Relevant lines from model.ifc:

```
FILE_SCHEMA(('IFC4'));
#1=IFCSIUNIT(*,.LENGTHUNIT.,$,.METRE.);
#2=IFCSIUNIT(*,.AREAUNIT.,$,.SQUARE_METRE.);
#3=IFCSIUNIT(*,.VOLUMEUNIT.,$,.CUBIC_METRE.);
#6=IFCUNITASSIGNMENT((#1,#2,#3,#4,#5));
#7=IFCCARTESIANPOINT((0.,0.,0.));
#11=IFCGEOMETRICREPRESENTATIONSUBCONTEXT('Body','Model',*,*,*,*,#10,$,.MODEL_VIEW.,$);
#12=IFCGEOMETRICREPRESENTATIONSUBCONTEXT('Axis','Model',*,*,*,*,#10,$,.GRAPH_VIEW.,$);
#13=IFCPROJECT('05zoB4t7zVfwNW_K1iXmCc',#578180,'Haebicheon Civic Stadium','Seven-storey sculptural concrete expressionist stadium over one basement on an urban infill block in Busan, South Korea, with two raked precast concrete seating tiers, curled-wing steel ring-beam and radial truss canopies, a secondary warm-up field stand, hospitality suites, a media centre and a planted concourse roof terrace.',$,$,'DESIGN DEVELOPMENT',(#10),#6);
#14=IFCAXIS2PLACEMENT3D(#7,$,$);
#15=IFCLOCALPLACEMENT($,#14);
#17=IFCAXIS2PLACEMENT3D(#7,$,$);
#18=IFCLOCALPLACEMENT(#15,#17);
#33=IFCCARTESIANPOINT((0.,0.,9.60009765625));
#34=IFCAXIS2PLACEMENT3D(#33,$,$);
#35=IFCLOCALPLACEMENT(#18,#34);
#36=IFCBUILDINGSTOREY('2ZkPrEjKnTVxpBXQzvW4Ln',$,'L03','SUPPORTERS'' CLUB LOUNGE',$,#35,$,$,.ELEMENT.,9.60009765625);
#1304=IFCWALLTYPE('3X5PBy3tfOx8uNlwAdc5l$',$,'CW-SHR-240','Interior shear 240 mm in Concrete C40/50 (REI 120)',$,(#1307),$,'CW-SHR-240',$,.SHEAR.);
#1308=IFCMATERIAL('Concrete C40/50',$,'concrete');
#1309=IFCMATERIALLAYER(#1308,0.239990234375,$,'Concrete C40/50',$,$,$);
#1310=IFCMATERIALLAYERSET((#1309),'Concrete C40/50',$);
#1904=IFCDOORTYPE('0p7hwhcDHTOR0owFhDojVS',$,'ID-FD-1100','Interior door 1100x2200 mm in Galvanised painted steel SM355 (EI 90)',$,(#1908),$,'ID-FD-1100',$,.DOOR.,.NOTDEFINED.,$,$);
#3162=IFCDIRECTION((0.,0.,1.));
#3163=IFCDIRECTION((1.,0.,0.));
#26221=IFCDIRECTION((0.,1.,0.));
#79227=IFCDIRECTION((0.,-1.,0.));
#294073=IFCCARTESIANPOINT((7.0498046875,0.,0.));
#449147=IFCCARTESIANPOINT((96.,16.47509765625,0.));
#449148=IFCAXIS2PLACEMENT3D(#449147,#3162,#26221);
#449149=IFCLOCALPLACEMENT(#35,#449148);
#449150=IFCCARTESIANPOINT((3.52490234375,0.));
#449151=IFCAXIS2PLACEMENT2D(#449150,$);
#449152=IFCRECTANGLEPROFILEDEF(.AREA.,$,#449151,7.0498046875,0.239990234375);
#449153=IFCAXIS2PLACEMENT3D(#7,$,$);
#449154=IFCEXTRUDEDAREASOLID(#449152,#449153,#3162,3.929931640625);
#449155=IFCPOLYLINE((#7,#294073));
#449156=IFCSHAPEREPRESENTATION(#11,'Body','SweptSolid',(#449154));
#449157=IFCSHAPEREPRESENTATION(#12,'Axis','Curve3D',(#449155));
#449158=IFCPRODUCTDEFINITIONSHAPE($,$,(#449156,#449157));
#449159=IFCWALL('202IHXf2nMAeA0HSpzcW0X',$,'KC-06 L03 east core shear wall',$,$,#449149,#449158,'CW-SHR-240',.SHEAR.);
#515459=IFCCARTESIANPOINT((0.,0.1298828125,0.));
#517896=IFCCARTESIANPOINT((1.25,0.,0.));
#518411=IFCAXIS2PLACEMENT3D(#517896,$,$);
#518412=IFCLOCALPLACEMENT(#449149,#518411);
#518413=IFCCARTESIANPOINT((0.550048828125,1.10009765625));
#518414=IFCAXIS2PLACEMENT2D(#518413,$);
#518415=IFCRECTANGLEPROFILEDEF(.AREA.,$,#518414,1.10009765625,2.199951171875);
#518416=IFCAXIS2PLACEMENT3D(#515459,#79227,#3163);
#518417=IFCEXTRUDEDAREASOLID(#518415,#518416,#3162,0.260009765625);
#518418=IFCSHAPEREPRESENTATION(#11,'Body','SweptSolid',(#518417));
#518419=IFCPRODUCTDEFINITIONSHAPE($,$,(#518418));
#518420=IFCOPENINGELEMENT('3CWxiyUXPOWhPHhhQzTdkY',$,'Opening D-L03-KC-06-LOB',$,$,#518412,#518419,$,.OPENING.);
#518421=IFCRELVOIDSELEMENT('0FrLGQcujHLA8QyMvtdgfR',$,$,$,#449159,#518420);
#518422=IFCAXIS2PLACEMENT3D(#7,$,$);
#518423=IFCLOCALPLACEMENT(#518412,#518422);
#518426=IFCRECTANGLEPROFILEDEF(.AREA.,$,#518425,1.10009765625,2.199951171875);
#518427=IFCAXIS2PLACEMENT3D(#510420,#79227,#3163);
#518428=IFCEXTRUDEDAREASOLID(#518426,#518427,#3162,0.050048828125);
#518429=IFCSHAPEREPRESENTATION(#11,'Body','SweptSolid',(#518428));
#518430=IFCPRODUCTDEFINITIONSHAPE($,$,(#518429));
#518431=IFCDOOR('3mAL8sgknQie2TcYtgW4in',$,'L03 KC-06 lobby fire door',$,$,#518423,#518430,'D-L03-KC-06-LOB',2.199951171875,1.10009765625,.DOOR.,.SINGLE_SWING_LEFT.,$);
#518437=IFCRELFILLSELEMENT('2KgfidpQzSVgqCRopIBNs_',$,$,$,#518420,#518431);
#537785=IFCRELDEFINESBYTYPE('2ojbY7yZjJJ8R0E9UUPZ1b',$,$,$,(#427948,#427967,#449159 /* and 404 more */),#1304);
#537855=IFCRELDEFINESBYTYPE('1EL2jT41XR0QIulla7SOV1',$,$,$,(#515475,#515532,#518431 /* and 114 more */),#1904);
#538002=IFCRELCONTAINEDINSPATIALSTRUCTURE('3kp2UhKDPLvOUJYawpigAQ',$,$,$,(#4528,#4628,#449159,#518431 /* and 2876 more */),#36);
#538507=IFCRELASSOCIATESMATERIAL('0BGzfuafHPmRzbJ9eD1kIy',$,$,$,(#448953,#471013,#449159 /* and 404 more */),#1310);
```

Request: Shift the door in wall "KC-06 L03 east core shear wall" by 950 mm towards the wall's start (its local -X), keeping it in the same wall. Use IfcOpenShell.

```python
import ifcopenshell
import ifcopenshell.api.geometry
import ifcopenshell.util.placement

model = ifcopenshell.open("model.ifc")

door = model.by_guid("3mAL8sgknQie2TcYtgW4in")
opening = door.FillsVoids[0].RelatingOpeningElement
wall = opening.VoidsElements[0].RelatingBuildingElement

wall_matrix = ifcopenshell.util.placement.get_local_placement(wall.ObjectPlacement)
shift = wall_matrix[:3, 0] * -0.95
before = ifcopenshell.util.placement.get_local_placement(door.ObjectPlacement)[:3, 3].copy()

# The door is placed relative to its opening, so it follows when the opening moves.
matrix = ifcopenshell.util.placement.get_local_placement(opening.ObjectPlacement)
matrix[:3, 3] += shift
ifcopenshell.api.geometry.edit_object_placement(
    model, product=opening, matrix=matrix, is_si=False, should_transform_children=True
)

after = ifcopenshell.util.placement.get_local_placement(door.ObjectPlacement)[:3, 3]
print("door moved by", (after - before).round(3) + 0.0)

model.write("model_edited.ifc")
```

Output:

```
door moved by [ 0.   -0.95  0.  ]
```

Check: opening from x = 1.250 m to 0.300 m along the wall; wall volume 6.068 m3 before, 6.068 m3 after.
